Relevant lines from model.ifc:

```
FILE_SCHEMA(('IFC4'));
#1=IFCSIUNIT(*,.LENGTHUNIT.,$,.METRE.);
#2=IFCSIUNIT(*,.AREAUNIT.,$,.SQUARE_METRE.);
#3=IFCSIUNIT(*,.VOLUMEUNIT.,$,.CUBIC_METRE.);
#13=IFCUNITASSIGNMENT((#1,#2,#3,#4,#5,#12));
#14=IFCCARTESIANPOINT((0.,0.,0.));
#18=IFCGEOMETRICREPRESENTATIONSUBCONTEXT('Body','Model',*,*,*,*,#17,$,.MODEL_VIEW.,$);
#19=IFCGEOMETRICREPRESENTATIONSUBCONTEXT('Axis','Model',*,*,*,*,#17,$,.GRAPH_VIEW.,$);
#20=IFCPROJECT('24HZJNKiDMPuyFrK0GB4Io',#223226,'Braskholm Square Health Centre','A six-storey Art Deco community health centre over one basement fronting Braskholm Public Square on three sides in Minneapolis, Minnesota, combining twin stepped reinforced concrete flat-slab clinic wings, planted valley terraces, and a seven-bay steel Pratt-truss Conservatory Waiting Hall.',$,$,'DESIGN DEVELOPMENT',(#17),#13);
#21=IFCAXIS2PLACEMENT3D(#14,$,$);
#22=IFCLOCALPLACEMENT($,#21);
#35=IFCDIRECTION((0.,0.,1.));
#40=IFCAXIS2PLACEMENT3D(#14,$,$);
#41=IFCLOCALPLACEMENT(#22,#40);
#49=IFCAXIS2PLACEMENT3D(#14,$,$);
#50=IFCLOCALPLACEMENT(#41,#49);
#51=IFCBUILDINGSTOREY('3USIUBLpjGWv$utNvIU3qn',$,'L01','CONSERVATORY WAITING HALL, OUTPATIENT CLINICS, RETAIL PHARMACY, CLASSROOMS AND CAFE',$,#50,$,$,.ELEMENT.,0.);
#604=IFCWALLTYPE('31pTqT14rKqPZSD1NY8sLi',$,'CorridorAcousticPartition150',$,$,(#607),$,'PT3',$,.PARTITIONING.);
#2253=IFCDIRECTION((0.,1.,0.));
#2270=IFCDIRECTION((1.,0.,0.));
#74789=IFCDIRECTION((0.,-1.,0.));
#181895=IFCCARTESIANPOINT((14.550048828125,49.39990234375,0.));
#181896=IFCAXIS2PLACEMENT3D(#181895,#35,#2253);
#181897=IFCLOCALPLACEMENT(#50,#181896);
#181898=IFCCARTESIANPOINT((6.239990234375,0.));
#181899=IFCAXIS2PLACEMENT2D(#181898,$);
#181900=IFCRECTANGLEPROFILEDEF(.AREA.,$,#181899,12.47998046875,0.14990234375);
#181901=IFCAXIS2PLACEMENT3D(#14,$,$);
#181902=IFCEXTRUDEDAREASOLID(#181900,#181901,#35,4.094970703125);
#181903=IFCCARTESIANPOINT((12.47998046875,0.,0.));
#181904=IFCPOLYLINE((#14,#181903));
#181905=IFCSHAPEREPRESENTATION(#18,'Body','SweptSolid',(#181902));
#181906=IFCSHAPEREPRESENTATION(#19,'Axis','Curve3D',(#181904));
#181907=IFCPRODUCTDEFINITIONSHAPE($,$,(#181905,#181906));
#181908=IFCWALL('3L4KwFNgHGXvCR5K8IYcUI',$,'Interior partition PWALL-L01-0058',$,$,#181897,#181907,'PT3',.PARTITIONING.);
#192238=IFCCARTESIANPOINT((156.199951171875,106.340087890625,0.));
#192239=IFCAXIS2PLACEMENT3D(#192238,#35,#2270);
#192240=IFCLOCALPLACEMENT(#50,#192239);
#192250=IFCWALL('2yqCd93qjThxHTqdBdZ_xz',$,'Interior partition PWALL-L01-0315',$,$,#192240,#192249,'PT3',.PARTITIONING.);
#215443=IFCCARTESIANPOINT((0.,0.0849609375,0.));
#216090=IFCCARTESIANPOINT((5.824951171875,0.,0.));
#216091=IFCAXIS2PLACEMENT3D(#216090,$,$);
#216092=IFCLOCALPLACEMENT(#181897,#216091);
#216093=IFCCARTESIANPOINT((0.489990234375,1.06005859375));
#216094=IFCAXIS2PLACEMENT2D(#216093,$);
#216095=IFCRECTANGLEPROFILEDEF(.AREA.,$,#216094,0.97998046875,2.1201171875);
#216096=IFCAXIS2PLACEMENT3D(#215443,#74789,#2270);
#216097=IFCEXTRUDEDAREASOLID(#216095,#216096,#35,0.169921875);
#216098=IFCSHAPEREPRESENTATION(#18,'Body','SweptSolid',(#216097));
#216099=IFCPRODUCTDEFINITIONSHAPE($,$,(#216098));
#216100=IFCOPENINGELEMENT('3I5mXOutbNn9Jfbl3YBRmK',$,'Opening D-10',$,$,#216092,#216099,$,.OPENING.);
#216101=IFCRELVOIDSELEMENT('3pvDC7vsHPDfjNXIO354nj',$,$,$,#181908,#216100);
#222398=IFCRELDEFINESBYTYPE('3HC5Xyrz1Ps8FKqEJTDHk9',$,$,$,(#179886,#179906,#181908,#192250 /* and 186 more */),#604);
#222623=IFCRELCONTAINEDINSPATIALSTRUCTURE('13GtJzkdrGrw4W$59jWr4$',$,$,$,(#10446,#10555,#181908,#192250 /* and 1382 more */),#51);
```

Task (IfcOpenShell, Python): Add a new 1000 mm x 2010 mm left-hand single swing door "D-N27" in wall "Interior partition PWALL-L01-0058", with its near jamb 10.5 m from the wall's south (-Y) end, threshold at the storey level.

```python
import numpy as np
import ifcopenshell
import ifcopenshell.api.feature
import ifcopenshell.api.geometry
import ifcopenshell.api.root
import ifcopenshell.api.spatial
import ifcopenshell.geom
import ifcopenshell.util.element
import ifcopenshell.util.placement
import ifcopenshell.util.representation
import ifcopenshell.util.shape
import ifcopenshell.util.unit

model = ifcopenshell.open("model.ifc")
unit_scale = ifcopenshell.util.unit.calculate_unit_scale(model)
settings = ifcopenshell.geom.settings()


def volume(element):
    """Net volume in cubic metres, openings subtracted."""
    shape = ifcopenshell.geom.create_shape(settings, element)
    return ifcopenshell.util.shape.get_volume(shape.geometry)


wall = model.by_guid("3L4KwFNgHGXvCR5K8IYcUI")
storey = ifcopenshell.util.element.get_container(wall, ifc_class="IfcBuildingStorey")
context = ifcopenshell.util.representation.get_context(model, "Model", "Body", "MODEL_VIEW")
before = volume(wall)

width, height, from_end, sill = 1, 2.01, 10.5, 0.0  # metres

# The wall runs along its own X axis, and the end named is its -X end.
wall_shape = ifcopenshell.geom.create_shape(settings, wall)
x, y, z = ifcopenshell.util.shape.get_vertices(wall_shape.geometry).T
start = x.min() + from_end
face, thickness = float(y.min()), float(y.max() - y.min())
wall_matrix = ifcopenshell.util.placement.get_local_placement(wall.ObjectPlacement)
level = ifcopenshell.util.placement.get_local_placement(storey.ObjectPlacement)[2, 3]


def in_wall(x, y):
    """Placement at x, y metres in the wall's axes, at sill height."""
    matrix = wall_matrix.copy()
    matrix[:, 3] = wall_matrix @ np.array([x / unit_scale, y / unit_scale, 0.0, 1.0])
    matrix[2, 3] = level + sill / unit_scale
    return matrix


# Opening: a box that overshoots both wall faces by 50 mm.
opening = ifcopenshell.api.root.create_entity(model, ifc_class="IfcOpeningElement", predefined_type="OPENING")
box = ifcopenshell.api.geometry.add_wall_representation(
    model, context=context, length=width, height=height, thickness=thickness + 0.1
)
ifcopenshell.api.geometry.assign_representation(model, product=opening, representation=box)
ifcopenshell.api.geometry.edit_object_placement(model, product=opening, matrix=in_wall(start, face - 0.05), is_si=False)
ifcopenshell.api.feature.add_feature(model, feature=opening, element=wall)

door = ifcopenshell.api.root.create_entity(model, ifc_class="IfcDoor", name="D-N27", predefined_type="DOOR")
door.OverallWidth, door.OverallHeight = width / unit_scale, height / unit_scale
door.OperationType = "SINGLE_SWING_LEFT"
body = ifcopenshell.api.geometry.add_door_representation(
    model,
    context=context,
    overall_width=door.OverallWidth,
    overall_height=door.OverallHeight,
    operation_type="SINGLE_SWING_LEFT",
    lining_properties={"LiningDepth": thickness / unit_scale, "ThresholdDepth": thickness / unit_scale},
)
ifcopenshell.api.geometry.assign_representation(model, product=door, representation=body)
ifcopenshell.api.spatial.assign_container(model, products=[door], relating_structure=storey)
ifcopenshell.api.feature.add_filling(model, opening=opening, element=door)

# The lining spans the wall, so the door starts at the wall face.
ifcopenshell.api.geometry.edit_object_placement(model, product=door, matrix=in_wall(start, face), is_si=False)

after = volume(wall)

print(f"wall volume {before:.3f} -> {after:.3f} m3")

model.write("model_rev.ifc")
```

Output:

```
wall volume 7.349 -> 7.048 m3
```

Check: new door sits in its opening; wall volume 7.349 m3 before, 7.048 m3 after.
